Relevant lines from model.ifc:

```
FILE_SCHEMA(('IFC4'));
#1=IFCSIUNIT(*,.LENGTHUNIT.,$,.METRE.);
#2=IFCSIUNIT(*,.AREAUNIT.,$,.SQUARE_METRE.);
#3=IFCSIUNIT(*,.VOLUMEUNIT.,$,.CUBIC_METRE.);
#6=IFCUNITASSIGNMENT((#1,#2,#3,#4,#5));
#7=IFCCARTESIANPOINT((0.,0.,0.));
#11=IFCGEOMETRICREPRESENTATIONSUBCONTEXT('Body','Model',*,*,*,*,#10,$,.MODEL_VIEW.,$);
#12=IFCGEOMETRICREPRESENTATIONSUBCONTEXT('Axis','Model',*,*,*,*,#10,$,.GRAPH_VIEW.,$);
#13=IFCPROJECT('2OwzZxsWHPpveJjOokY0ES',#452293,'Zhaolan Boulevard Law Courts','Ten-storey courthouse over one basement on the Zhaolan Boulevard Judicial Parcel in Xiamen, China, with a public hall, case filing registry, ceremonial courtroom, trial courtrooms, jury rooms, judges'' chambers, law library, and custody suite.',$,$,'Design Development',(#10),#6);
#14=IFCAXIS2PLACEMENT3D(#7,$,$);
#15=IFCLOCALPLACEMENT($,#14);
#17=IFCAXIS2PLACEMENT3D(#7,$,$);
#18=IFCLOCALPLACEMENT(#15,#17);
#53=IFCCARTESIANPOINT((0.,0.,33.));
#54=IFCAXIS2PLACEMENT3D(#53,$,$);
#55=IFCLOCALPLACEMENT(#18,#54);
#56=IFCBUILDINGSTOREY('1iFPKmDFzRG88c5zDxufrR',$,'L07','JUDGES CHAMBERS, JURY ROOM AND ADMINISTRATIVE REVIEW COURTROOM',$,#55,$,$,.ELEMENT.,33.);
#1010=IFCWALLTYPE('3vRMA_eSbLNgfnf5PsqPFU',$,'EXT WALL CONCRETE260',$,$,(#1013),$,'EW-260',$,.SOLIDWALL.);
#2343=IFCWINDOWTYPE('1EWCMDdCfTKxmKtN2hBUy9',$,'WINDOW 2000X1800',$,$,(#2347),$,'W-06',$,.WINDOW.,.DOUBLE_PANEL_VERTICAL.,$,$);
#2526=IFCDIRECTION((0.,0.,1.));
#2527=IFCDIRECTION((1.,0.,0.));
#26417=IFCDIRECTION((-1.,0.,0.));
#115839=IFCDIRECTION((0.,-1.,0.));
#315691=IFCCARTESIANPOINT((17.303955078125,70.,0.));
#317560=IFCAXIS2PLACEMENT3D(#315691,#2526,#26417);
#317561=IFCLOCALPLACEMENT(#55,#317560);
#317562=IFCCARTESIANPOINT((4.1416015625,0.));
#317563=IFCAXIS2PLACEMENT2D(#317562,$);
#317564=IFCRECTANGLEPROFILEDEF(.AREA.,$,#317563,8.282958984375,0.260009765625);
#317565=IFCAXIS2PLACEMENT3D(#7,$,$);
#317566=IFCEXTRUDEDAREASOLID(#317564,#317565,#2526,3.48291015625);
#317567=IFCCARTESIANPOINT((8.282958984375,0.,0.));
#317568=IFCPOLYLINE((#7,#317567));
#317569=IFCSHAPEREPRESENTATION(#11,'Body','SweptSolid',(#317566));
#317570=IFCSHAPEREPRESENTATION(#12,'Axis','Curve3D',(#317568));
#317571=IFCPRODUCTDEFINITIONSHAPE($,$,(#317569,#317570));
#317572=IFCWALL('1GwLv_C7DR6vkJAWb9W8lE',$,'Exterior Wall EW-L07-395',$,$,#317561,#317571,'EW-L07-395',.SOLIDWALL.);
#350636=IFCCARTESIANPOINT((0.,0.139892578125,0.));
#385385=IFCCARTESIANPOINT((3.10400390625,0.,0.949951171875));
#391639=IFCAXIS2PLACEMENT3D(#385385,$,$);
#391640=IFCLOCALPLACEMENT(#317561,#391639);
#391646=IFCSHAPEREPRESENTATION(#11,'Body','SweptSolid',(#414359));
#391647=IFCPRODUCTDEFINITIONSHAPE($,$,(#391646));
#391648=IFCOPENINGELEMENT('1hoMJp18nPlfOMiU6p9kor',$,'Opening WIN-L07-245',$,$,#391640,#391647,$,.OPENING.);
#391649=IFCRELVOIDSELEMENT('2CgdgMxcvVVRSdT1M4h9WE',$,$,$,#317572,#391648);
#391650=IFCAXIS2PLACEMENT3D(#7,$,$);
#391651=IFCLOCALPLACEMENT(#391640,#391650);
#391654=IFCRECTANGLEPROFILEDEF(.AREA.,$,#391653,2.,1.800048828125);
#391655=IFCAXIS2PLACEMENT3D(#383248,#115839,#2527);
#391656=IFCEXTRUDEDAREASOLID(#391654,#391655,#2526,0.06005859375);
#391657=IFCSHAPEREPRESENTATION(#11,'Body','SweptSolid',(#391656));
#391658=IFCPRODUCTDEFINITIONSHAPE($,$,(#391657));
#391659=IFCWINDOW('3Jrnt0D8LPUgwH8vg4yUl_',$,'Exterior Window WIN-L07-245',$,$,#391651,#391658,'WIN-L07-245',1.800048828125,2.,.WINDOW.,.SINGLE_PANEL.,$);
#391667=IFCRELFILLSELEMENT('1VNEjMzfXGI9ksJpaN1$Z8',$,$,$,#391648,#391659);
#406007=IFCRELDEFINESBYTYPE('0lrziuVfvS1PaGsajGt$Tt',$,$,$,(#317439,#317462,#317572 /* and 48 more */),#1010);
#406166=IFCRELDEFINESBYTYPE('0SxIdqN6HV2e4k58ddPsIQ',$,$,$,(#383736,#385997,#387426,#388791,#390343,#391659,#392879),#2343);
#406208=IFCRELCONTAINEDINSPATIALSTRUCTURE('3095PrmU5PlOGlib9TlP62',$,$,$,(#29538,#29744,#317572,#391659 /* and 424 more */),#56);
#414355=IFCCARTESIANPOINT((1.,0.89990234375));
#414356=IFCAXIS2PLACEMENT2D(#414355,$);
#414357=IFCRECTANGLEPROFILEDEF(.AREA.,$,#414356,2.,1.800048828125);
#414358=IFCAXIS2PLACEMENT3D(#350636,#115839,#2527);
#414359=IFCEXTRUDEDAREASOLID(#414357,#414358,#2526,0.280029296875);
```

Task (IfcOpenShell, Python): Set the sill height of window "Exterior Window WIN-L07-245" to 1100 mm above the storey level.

```python
import numpy as np
import ifcopenshell
import ifcopenshell.api.geometry
import ifcopenshell.geom
import ifcopenshell.util.element
import ifcopenshell.util.placement
import ifcopenshell.util.shape
import ifcopenshell.util.unit

model = ifcopenshell.open("model.ifc")
unit_scale = ifcopenshell.util.unit.calculate_unit_scale(model)

window = model.by_guid("3Jrnt0D8LPUgwH8vg4yUl_")
opening = window.FillsVoids[0].RelatingOpeningElement
storey = ifcopenshell.util.element.get_container(window, ifc_class="IfcBuildingStorey")
level = ifcopenshell.util.placement.get_local_placement(storey.ObjectPlacement)[2, 3]

# The opening's origin need not be at the sill, so measure its lowest point.
shape = ifcopenshell.geom.create_shape(ifcopenshell.geom.settings(), opening)
bottom = ifcopenshell.util.shape.get_shape_bottom_elevation(shape, shape.geometry) / unit_scale
dz = level + 1.1 / unit_scale - bottom

shift = np.array([0.0, 0.0, dz])
# The window is placed relative to its opening, so it follows when the opening moves.
matrix = ifcopenshell.util.placement.get_local_placement(opening.ObjectPlacement)
matrix[:3, 3] += shift
ifcopenshell.api.geometry.edit_object_placement(
    model, product=opening, matrix=matrix, is_si=False, should_transform_children=True
)

print(f"moved by {dz * unit_scale:+.3f} m")

model.write("model_updated.ifc")
```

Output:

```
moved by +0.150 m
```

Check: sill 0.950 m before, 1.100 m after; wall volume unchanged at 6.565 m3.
